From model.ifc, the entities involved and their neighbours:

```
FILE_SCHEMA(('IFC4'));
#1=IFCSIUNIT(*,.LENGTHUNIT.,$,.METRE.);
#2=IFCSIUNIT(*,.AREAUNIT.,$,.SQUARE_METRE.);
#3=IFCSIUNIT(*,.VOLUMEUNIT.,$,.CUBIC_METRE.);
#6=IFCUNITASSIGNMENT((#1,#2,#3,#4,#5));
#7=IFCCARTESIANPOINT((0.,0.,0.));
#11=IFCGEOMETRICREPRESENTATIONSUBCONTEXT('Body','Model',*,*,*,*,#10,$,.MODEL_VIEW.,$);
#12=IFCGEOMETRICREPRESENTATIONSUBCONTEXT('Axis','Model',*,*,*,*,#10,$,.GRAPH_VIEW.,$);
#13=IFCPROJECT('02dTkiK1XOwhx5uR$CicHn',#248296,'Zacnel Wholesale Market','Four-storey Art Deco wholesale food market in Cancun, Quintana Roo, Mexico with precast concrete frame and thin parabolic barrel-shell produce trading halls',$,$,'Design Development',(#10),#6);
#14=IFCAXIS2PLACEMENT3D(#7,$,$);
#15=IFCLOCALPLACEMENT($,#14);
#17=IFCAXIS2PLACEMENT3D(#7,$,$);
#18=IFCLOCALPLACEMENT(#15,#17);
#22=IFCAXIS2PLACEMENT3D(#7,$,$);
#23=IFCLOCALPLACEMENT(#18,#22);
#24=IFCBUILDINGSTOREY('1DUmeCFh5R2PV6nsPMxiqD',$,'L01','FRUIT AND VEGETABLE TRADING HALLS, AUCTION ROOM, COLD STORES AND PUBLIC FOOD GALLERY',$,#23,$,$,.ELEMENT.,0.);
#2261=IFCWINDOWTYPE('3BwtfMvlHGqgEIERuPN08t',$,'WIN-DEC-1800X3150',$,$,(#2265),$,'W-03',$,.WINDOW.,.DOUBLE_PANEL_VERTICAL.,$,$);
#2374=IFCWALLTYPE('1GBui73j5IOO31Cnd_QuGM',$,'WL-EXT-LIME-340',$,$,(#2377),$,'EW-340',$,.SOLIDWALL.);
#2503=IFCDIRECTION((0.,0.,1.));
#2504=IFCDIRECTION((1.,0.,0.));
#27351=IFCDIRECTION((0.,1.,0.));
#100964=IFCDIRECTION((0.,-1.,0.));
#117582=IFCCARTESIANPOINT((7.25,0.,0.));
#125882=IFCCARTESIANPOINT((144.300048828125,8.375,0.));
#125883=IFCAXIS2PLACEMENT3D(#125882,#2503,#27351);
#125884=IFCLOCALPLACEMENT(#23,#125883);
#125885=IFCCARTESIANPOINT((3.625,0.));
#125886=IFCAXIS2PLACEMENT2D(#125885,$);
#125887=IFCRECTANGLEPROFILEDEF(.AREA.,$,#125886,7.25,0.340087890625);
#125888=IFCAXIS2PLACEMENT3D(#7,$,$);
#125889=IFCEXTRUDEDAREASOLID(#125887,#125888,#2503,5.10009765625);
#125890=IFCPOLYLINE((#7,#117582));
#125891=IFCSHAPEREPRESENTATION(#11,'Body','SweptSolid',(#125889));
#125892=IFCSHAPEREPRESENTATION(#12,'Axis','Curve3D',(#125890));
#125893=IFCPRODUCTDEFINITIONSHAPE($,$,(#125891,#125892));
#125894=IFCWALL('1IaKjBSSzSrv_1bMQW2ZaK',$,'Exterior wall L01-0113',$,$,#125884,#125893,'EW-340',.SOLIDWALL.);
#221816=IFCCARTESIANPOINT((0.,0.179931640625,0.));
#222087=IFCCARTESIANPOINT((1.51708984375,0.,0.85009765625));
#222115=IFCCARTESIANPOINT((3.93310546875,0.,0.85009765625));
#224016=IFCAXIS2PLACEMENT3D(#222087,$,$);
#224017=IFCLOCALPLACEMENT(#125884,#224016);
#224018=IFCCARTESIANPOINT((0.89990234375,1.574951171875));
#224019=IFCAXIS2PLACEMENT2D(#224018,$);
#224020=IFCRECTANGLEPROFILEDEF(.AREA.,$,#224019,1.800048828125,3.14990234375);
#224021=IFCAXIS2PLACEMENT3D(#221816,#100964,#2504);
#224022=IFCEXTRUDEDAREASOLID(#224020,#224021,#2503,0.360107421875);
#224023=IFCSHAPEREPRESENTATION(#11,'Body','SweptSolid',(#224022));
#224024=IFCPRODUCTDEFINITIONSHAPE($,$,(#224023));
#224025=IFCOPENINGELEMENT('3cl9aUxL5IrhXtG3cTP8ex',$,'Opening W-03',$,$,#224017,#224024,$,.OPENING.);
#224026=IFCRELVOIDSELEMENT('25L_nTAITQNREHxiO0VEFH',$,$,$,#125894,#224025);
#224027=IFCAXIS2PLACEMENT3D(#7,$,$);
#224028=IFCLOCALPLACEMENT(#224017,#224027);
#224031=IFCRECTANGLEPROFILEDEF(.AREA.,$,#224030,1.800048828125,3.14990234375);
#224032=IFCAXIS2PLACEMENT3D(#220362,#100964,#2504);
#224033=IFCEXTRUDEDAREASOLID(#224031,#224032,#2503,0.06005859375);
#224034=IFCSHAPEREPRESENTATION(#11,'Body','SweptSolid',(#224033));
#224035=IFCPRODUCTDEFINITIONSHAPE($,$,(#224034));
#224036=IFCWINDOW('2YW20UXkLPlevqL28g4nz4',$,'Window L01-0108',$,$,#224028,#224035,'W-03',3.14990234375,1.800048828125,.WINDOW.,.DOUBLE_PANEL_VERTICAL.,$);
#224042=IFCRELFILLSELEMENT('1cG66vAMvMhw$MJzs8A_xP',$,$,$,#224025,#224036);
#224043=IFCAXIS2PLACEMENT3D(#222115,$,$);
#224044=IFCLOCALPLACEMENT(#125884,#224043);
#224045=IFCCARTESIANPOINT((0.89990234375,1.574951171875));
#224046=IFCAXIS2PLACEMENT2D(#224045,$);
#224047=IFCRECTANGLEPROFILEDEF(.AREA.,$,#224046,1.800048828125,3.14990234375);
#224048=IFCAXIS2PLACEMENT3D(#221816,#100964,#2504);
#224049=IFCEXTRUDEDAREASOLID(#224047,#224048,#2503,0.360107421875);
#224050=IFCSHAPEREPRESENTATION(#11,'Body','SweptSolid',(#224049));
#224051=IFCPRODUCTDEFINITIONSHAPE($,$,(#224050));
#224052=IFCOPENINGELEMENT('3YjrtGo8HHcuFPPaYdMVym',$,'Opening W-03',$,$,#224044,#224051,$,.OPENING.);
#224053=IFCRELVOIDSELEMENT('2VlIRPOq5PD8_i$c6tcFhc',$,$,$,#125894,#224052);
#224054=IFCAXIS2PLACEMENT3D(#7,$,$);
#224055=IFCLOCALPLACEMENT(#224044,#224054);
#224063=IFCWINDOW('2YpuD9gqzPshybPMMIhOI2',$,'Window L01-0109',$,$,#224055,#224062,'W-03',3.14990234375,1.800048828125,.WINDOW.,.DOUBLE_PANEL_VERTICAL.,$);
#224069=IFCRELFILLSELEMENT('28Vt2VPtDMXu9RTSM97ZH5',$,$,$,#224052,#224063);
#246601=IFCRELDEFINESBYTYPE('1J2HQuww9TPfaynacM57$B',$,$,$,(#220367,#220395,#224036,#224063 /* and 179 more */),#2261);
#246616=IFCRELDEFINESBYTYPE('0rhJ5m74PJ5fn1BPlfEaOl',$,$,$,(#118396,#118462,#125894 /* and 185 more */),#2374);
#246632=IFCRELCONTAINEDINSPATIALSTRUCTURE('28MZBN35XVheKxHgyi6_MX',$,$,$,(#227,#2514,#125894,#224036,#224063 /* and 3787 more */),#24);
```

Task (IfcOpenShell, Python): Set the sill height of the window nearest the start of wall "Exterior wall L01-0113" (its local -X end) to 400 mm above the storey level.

```python
import numpy as np
import ifcopenshell
import ifcopenshell.api.geometry
import ifcopenshell.geom
import ifcopenshell.util.element
import ifcopenshell.util.placement
import ifcopenshell.util.shape
import ifcopenshell.util.unit

model = ifcopenshell.open("model.ifc")
unit_scale = ifcopenshell.util.unit.calculate_unit_scale(model)

window = model.by_guid("2YW20UXkLPlevqL28g4nz4")
opening = window.FillsVoids[0].RelatingOpeningElement
storey = ifcopenshell.util.element.get_container(window, ifc_class="IfcBuildingStorey")
level = ifcopenshell.util.placement.get_local_placement(storey.ObjectPlacement)[2, 3]

# The opening's origin need not be at the sill, so measure its lowest point.
shape = ifcopenshell.geom.create_shape(ifcopenshell.geom.settings(), opening)
bottom = ifcopenshell.util.shape.get_shape_bottom_elevation(shape, shape.geometry) / unit_scale
dz = level + 0.4 - bottom

shift = np.array([0.0, 0.0, dz])
# The window is placed relative to its opening, so it follows when the opening moves.
matrix = ifcopenshell.util.placement.get_local_placement(opening.ObjectPlacement)
matrix[:3, 3] += shift
ifcopenshell.api.geometry.edit_object_placement(
    model, product=opening, matrix=matrix, is_si=False, should_transform_children=True
)

print(f"moved by {dz * unit_scale:+.3f} m")

model.write("model_v2.ifc")
```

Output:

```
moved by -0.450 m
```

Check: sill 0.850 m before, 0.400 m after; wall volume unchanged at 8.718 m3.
